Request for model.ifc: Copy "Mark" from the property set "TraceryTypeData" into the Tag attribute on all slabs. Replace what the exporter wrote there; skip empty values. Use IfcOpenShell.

First a look at what the model holds.

```python
import ifcopenshell
import ifcopenshell.util.element

model = ifcopenshell.open("model.ifc")
print(model.schema)
slabs = model.by_type("IfcSlab")
print(len(slabs), "slabs")
for e in slabs[:8]:
    source = ifcopenshell.util.element.get_pset(e, "TraceryTypeData", "Mark")
    target = e.Tag
    print(e.id(), repr(source), repr(target), sep=" | ")
```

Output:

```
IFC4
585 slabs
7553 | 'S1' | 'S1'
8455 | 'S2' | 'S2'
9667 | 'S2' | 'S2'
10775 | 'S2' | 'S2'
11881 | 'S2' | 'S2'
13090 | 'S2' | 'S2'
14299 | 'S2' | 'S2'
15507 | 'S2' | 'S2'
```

```python
import ifcopenshell
import ifcopenshell.util.element

model = ifcopenshell.open("model.ifc")

count = 0
for e in model.by_type("IfcSlab"):
    value = ifcopenshell.util.element.get_pset(e, "TraceryTypeData", "Mark")
    current = e.Tag
    if not value or not value.strip() or current == value:
        continue
    e.Tag = value
    count += 1

print(count, "slabs updated")

model.write("model_rev.ifc")
```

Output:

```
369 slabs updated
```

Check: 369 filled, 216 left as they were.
